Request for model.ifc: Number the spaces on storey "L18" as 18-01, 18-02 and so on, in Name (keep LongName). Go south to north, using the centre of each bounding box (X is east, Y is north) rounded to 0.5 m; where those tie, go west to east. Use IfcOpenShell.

First a look at what the model holds.

```python
import ifcopenshell
import ifcopenshell.util.element
import ifcopenshell.util.placement

model = ifcopenshell.open("model.ifc")
print(model.schema)
storey = next(s for s in model.by_type("IfcBuildingStorey") if s.Name == "L18")
spaces = [e for e in ifcopenshell.util.element.get_decomposition(storey) if e.is_a("IfcSpace")]
for e in sorted(spaces, key=lambda e: e.id()):
    origin = ifcopenshell.util.placement.get_local_placement(e.ObjectPlacement)[:3, 3]
    print(e.id(), e.Name, e.LongName, origin.round(2) + 0.0, sep=" | ")
```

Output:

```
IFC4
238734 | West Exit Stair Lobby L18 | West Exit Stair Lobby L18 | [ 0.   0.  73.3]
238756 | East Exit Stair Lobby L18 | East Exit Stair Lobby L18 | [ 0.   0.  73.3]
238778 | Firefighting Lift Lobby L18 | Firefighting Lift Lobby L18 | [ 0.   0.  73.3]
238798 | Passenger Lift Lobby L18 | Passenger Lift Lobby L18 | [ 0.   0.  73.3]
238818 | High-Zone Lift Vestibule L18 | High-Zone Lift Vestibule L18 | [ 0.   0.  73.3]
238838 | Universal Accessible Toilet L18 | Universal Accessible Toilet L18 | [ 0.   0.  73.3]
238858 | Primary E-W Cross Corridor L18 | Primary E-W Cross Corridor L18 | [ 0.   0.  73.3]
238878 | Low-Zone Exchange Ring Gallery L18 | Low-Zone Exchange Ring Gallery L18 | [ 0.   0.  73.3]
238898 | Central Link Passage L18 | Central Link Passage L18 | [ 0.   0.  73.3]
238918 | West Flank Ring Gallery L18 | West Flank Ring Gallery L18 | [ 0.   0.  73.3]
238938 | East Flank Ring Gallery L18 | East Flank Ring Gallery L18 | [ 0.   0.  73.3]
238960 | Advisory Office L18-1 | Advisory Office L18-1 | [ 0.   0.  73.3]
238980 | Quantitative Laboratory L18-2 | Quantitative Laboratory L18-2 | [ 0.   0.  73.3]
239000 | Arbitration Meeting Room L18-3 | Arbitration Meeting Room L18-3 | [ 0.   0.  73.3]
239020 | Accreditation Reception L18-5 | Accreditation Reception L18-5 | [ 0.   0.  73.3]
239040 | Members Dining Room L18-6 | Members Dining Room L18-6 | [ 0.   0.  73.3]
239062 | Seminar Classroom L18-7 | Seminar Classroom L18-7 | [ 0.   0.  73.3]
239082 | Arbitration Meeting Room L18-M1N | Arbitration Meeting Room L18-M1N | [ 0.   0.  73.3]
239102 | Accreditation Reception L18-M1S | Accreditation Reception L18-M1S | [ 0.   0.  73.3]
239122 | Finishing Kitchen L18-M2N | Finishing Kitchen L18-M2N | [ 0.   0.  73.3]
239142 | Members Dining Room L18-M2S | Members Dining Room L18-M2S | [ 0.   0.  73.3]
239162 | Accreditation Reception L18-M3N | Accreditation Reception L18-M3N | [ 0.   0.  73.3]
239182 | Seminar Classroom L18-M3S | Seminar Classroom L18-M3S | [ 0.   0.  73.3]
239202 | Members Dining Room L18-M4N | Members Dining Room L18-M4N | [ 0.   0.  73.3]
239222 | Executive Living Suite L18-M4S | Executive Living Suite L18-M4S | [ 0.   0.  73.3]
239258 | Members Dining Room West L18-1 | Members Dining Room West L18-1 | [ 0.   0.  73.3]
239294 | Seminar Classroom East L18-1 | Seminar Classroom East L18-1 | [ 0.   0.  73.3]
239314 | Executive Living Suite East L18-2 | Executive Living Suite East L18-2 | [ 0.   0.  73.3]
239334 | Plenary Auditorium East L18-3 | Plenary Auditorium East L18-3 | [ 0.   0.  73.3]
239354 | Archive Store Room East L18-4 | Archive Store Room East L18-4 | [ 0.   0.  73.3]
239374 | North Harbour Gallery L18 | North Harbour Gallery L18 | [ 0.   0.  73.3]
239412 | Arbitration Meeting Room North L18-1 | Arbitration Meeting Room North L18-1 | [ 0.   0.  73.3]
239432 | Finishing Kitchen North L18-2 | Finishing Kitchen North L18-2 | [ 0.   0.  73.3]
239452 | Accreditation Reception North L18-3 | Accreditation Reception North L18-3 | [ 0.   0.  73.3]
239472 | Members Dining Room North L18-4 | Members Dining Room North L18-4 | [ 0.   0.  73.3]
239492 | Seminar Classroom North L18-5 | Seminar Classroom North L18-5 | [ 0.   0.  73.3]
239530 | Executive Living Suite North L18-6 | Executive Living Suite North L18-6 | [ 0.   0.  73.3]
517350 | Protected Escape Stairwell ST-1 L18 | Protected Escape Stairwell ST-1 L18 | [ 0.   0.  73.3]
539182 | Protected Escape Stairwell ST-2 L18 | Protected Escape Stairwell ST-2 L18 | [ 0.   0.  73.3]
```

```python
import ifcopenshell
import ifcopenshell.geom
import ifcopenshell.util.element
import ifcopenshell.util.shape

model = ifcopenshell.open("model.ifc")
settings = ifcopenshell.geom.settings()
settings.set("use-world-coords", True)


def centre(element):
    shape = ifcopenshell.geom.create_shape(settings, element)
    return ifcopenshell.util.shape.get_bbox_centroid(shape.geometry)


storey = next(s for s in model.by_type("IfcBuildingStorey") if s.Name == "L18")
spaces = [e for e in ifcopenshell.util.element.get_decomposition(storey) if e.is_a("IfcSpace")]

# Insertion points can sit at a corner or the storey origin, so sort by the geometry (in metres).
centres = {e: centre(e) for e in spaces}
spaces.sort(key=lambda e: (round(centres[e][1] / 0.5), centres[e][0]))

for i, e in enumerate(spaces, start=1):
    number = f"18-{i:02d}"
    e.Name = number
    print(e.id(), number)

model.write("model_edited.ifc")
```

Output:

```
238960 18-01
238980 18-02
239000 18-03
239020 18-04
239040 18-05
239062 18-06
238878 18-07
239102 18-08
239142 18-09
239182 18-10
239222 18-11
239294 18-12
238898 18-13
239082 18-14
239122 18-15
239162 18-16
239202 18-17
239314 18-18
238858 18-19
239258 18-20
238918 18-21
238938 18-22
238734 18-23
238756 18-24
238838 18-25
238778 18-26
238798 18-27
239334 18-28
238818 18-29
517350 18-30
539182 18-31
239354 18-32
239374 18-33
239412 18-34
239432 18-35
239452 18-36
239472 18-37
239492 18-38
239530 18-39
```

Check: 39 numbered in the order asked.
